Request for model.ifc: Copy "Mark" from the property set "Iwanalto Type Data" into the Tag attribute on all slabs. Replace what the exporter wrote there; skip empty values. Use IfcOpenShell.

First a look at what the model holds.

```python
import ifcopenshell
import ifcopenshell.util.element

model = ifcopenshell.open("model.ifc")
print(model.schema)
slabs = model.by_type("IfcSlab")
print(len(slabs), "slabs")
for e in slabs[:8]:
    source = ifcopenshell.util.element.get_pset(e, "Iwanalto Type Data", "Mark")
    target = e.Tag
    print(e.id(), repr(source), repr(target), sep=" | ")
```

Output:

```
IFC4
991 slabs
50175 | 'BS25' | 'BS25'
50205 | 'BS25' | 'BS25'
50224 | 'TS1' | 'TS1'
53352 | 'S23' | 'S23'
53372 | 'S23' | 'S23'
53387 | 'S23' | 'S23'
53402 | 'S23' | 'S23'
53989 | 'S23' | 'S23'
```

```python
import ifcopenshell
import ifcopenshell.util.element

model = ifcopenshell.open("model.ifc")

count = 0
for e in model.by_type("IfcSlab"):
    value = ifcopenshell.util.element.get_pset(e, "Iwanalto Type Data", "Mark")
    current = e.Tag
    if not value or not value.strip() or current == value:
        continue
    e.Tag = value
    count += 1

print(count, "slabs updated")

model.write("model_v2.ifc")
```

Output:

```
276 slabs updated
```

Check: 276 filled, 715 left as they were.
